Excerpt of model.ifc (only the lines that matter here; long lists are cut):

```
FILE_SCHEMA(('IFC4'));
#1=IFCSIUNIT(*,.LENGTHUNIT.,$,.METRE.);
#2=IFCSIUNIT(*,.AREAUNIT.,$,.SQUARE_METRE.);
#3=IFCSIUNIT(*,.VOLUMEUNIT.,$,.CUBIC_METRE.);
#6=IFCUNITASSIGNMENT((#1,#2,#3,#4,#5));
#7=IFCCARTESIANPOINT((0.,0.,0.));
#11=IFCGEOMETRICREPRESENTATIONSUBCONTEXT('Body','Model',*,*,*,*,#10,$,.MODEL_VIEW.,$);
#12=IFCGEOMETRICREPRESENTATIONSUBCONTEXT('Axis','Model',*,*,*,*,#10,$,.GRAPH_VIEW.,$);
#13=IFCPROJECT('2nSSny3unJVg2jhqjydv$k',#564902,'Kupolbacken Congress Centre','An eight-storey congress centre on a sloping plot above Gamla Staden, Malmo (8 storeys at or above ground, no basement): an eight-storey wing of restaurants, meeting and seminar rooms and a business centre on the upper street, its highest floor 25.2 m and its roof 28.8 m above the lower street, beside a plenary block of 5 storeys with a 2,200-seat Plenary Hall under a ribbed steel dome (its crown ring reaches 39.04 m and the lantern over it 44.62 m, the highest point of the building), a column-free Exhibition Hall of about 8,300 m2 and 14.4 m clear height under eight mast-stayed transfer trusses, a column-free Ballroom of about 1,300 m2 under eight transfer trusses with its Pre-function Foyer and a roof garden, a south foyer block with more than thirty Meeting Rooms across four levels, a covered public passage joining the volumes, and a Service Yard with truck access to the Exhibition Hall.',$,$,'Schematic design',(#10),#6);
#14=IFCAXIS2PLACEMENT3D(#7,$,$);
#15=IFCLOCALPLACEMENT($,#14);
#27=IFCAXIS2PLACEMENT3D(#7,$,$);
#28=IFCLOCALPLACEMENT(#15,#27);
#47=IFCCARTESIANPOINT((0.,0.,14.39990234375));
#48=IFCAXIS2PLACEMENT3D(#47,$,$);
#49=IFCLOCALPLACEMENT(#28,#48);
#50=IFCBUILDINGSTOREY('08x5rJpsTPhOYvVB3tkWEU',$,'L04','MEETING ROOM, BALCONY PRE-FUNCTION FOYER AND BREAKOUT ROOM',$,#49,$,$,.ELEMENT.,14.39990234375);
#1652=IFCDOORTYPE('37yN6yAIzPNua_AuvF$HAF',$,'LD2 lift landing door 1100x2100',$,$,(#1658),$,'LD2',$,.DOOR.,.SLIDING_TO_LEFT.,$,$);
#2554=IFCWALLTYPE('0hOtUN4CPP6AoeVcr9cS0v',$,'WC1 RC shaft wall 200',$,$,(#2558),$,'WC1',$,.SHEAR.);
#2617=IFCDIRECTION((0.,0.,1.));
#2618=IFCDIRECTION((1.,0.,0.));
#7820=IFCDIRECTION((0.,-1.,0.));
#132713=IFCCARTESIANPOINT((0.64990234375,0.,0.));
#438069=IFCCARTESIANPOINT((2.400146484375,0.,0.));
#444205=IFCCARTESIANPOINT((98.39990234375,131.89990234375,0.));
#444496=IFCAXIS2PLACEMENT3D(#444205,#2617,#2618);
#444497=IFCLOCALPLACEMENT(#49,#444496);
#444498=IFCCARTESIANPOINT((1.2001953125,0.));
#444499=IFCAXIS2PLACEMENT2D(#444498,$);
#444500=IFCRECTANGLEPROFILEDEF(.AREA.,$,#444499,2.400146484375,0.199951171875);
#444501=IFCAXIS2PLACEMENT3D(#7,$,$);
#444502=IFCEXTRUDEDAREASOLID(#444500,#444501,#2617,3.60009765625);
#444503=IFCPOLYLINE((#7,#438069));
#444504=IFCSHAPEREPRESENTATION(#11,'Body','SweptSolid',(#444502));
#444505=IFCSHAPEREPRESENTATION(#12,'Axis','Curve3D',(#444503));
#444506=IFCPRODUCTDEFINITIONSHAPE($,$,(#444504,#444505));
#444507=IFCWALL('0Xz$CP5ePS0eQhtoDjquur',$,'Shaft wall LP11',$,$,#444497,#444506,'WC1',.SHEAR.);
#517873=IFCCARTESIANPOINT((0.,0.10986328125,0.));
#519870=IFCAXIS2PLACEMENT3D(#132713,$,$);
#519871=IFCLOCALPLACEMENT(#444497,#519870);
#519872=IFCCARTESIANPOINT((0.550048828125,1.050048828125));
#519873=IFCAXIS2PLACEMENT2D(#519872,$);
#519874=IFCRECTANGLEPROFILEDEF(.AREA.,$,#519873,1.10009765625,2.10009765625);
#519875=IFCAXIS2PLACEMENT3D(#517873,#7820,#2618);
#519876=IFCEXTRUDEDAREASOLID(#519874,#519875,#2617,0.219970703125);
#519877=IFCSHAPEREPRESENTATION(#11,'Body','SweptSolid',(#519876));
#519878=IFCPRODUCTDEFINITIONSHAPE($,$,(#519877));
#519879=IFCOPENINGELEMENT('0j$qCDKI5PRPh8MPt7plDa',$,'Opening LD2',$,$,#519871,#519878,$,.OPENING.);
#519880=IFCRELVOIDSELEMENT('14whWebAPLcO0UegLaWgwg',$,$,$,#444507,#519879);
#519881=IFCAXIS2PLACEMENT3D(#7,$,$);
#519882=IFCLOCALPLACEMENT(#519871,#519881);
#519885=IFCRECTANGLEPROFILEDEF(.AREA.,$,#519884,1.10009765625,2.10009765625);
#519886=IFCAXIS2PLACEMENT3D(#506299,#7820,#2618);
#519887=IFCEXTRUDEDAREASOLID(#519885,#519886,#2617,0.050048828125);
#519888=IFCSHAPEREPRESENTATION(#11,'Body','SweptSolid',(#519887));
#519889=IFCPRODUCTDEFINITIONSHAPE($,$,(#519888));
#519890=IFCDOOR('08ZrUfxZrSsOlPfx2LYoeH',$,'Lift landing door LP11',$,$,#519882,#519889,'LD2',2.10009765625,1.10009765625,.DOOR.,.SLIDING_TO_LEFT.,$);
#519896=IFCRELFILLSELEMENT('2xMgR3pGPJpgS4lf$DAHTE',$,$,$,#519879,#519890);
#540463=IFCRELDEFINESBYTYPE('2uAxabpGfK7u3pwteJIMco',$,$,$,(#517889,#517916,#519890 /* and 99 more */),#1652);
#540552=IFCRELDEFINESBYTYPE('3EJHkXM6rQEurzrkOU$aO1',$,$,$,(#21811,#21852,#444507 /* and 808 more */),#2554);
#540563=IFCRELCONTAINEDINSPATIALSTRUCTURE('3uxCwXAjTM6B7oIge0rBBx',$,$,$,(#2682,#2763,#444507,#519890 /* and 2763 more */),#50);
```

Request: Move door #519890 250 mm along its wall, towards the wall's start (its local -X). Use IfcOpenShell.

```python
import ifcopenshell
import ifcopenshell.api.geometry
import ifcopenshell.util.placement

model = ifcopenshell.open("model.ifc")

door = model.by_guid("08ZrUfxZrSsOlPfx2LYoeH")
opening = door.FillsVoids[0].RelatingOpeningElement
wall = opening.VoidsElements[0].RelatingBuildingElement

wall_matrix = ifcopenshell.util.placement.get_local_placement(wall.ObjectPlacement)
shift = wall_matrix[:3, 0] * -0.25
before = ifcopenshell.util.placement.get_local_placement(door.ObjectPlacement)[:3, 3].copy()

# The door is placed relative to its opening, so it follows when the opening moves.
matrix = ifcopenshell.util.placement.get_local_placement(opening.ObjectPlacement)
matrix[:3, 3] += shift
ifcopenshell.api.geometry.edit_object_placement(
    model, product=opening, matrix=matrix, is_si=False, should_transform_children=True
)

after = ifcopenshell.util.placement.get_local_placement(door.ObjectPlacement)[:3, 3]
print("door moved by", (after - before).round(3) + 0.0)

model.write("model-out.ifc")
```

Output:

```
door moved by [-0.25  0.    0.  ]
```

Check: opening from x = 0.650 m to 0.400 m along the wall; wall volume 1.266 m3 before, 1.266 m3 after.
